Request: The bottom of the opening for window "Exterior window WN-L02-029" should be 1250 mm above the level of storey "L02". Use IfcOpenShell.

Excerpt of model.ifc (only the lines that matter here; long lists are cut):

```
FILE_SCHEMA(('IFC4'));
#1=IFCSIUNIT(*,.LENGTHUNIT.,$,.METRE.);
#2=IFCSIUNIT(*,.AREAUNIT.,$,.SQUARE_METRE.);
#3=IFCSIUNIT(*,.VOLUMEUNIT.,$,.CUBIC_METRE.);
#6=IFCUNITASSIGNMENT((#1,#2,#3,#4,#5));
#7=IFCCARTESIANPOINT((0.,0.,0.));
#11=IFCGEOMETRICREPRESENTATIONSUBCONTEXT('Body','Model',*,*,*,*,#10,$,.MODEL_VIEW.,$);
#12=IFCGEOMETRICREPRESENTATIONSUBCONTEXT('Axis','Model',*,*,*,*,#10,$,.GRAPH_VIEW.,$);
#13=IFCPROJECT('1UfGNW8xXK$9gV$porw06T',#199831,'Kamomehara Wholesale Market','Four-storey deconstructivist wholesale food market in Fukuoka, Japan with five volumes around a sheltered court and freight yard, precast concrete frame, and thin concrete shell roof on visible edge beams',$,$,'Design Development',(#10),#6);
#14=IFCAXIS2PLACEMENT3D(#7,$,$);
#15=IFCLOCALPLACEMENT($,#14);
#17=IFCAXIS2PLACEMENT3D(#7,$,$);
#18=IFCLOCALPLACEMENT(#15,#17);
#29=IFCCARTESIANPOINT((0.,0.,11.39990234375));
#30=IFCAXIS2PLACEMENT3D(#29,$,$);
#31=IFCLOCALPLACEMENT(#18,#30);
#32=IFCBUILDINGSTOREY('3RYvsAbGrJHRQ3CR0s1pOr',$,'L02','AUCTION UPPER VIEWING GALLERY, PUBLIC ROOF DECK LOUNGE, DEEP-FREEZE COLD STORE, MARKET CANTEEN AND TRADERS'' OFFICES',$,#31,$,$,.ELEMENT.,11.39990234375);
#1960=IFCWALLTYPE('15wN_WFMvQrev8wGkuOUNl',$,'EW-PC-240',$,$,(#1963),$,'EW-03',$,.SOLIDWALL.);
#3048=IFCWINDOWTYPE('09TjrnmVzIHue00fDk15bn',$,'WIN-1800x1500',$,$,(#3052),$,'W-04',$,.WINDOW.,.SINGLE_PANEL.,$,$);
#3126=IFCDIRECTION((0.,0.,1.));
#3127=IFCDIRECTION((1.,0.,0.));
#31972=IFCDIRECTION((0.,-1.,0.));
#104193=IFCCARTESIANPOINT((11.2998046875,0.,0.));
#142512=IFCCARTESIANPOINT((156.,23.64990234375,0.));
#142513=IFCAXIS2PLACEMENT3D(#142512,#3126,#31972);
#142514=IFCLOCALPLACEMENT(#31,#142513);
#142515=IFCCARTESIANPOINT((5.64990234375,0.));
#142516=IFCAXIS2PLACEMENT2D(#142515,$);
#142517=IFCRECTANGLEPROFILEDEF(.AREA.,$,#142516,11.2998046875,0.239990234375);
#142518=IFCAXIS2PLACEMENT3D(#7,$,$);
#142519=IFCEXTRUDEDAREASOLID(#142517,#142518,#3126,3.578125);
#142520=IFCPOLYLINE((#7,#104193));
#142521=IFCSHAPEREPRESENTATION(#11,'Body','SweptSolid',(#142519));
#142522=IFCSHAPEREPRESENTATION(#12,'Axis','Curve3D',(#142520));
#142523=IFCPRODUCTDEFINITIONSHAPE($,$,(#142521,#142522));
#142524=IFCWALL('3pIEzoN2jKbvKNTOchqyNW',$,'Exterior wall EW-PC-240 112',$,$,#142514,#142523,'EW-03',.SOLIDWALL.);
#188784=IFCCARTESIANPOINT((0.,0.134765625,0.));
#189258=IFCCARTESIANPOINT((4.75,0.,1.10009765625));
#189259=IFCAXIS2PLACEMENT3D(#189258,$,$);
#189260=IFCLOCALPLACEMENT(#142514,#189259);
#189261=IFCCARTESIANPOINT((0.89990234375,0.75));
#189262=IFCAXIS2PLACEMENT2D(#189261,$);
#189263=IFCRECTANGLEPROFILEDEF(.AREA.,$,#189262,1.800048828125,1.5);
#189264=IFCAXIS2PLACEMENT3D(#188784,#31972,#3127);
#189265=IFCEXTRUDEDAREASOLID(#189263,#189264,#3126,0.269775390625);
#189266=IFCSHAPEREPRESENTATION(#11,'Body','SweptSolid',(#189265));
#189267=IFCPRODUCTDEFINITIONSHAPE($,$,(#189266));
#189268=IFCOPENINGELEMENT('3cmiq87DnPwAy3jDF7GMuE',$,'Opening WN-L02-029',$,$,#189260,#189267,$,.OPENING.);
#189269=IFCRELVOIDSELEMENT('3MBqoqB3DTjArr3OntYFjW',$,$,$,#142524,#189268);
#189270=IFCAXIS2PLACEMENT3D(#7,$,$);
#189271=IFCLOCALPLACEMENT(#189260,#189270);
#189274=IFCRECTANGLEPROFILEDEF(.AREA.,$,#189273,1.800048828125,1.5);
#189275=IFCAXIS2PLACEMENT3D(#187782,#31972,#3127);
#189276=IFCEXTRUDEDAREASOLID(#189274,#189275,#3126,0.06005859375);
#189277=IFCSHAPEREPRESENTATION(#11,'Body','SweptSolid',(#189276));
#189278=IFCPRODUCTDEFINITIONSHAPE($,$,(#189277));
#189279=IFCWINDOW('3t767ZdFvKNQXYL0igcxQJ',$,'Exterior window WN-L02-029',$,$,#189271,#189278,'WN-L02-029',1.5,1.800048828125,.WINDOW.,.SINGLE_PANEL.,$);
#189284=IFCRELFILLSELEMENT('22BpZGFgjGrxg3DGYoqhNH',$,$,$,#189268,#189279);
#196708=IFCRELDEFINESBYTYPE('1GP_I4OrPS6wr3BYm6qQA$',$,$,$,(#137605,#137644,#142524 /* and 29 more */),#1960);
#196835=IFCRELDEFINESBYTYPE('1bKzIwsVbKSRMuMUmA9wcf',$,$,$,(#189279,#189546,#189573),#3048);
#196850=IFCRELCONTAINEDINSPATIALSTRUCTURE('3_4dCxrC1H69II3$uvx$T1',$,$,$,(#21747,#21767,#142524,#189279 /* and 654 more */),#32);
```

```python
import numpy as np
import ifcopenshell
import ifcopenshell.api.geometry
import ifcopenshell.geom
import ifcopenshell.util.element
import ifcopenshell.util.placement
import ifcopenshell.util.shape
import ifcopenshell.util.unit

model = ifcopenshell.open("model.ifc")
unit_scale = ifcopenshell.util.unit.calculate_unit_scale(model)

window = model.by_guid("3t767ZdFvKNQXYL0igcxQJ")
opening = window.FillsVoids[0].RelatingOpeningElement
storey = ifcopenshell.util.element.get_container(window, ifc_class="IfcBuildingStorey")
level = ifcopenshell.util.placement.get_local_placement(storey.ObjectPlacement)[2, 3]

# The opening's origin need not be at the sill, so measure its lowest point.
shape = ifcopenshell.geom.create_shape(ifcopenshell.geom.settings(), opening)
bottom = ifcopenshell.util.shape.get_shape_bottom_elevation(shape, shape.geometry) / unit_scale
dz = level + 1.25 - bottom

shift = np.array([0.0, 0.0, dz])
# The window is placed relative to its opening, so it follows when the opening moves.
matrix = ifcopenshell.util.placement.get_local_placement(opening.ObjectPlacement)
matrix[:3, 3] += shift
ifcopenshell.api.geometry.edit_object_placement(
    model, product=opening, matrix=matrix, is_si=False, should_transform_children=True
)

print(f"moved by {dz * unit_scale:+.3f} m")

model.write("model_rev.ifc")
```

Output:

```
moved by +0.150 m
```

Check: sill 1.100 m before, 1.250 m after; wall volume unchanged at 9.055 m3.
